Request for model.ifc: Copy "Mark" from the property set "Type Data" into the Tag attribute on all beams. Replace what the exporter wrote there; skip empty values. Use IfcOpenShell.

First a look at what the model holds.

```python
import ifcopenshell
import ifcopenshell.util.element

model = ifcopenshell.open("model.ifc")
print(model.schema)
beams = model.by_type("IfcBeam")
print(len(beams), "beams")
for e in beams[:8]:
    source = ifcopenshell.util.element.get_pset(e, "Type Data", "Mark")
    target = e.Tag
    print(e.id(), repr(source), repr(target), sep=" | ")
```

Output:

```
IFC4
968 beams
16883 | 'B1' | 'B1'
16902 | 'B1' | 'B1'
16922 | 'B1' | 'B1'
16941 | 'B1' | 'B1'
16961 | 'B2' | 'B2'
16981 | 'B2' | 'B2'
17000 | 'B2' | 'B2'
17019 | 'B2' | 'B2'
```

```python
import ifcopenshell
import ifcopenshell.util.element

model = ifcopenshell.open("model.ifc")

count = 0
for e in model.by_type("IfcBeam"):
    value = ifcopenshell.util.element.get_pset(e, "Type Data", "Mark")
    current = e.Tag
    if not value or not value.strip() or current == value:
        continue
    e.Tag = value
    count += 1

print(count, "beams updated")

model.write("model_updated.ifc")
```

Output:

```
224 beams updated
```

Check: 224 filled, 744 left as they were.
